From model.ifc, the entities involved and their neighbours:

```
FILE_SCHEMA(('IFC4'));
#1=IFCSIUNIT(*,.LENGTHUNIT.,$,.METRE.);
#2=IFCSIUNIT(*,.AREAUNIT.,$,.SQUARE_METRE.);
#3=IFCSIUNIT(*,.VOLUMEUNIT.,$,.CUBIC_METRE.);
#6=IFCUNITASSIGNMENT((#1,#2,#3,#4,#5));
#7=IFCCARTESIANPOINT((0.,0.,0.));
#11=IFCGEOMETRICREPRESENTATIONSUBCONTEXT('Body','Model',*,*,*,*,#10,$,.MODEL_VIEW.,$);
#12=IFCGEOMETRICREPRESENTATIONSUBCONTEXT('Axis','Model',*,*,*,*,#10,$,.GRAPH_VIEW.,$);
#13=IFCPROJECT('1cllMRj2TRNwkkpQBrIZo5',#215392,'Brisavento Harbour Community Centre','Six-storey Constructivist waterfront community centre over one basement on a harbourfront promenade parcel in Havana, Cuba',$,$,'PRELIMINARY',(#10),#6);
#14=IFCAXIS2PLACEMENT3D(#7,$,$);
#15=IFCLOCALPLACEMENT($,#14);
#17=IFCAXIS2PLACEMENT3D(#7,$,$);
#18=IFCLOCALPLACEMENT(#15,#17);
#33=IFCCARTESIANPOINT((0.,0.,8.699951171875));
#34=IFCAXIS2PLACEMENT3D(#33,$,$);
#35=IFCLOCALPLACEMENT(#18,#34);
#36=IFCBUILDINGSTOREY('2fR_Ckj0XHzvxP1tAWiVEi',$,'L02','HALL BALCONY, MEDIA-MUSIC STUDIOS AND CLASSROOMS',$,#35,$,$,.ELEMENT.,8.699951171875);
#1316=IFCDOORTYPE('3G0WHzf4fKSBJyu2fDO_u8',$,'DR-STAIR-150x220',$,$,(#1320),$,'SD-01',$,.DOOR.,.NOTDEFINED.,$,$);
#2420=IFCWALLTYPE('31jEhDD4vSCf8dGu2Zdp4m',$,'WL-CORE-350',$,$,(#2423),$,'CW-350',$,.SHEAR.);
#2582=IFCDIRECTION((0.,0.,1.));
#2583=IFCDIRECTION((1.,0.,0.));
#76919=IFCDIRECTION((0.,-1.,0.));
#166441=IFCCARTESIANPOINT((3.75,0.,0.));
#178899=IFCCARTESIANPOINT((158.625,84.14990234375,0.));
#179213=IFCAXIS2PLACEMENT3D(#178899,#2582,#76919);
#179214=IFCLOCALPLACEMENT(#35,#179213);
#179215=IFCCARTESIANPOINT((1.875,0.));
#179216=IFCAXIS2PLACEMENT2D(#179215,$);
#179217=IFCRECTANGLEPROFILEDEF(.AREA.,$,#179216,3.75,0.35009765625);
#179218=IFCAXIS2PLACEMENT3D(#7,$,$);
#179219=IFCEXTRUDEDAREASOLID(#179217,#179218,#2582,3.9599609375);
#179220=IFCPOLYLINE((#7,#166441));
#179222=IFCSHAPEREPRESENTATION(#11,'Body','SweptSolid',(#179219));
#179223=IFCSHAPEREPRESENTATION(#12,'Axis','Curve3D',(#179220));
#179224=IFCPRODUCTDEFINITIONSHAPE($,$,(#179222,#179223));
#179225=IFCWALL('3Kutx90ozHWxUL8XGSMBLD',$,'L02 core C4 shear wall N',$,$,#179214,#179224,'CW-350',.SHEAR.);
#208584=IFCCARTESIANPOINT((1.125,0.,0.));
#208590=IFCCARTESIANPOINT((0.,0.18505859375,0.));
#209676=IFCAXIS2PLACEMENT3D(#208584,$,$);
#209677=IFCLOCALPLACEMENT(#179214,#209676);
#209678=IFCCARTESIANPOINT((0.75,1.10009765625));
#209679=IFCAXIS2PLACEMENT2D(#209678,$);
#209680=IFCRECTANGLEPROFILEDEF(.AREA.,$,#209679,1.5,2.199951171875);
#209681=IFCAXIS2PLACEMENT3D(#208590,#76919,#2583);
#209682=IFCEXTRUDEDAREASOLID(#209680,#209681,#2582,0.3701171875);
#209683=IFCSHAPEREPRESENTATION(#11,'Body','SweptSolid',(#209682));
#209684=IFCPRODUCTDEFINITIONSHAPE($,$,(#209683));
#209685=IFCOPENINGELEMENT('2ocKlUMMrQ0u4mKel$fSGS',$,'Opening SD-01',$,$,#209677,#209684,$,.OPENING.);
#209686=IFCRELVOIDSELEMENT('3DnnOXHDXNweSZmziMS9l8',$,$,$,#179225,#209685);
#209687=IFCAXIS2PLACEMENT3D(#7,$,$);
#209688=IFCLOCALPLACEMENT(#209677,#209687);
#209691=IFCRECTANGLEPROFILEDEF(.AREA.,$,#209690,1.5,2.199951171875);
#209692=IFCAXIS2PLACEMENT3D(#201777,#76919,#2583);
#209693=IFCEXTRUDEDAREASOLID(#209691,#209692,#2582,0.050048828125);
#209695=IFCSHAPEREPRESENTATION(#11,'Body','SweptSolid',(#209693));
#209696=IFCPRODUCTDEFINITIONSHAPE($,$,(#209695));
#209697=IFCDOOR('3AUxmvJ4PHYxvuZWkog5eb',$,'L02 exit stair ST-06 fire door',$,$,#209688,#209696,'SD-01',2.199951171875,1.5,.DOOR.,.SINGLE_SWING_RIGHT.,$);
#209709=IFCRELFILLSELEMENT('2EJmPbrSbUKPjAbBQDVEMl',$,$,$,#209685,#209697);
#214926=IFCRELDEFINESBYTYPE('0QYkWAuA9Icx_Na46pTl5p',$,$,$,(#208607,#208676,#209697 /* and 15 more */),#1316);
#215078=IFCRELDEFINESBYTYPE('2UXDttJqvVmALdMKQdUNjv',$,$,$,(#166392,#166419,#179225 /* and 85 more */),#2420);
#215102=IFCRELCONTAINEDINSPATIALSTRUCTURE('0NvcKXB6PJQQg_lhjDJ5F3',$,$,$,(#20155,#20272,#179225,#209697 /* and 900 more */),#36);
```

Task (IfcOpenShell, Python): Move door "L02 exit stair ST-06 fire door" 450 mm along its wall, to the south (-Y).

```python
import ifcopenshell
import ifcopenshell.api.geometry
import ifcopenshell.util.placement
import ifcopenshell.util.unit

model = ifcopenshell.open("model.ifc")
unit_scale = ifcopenshell.util.unit.calculate_unit_scale(model)

door = model.by_guid("3AUxmvJ4PHYxvuZWkog5eb")
opening = door.FillsVoids[0].RelatingOpeningElement
wall = opening.VoidsElements[0].RelatingBuildingElement

wall_matrix = ifcopenshell.util.placement.get_local_placement(wall.ObjectPlacement)
shift = wall_matrix[:3, 0] * 0.45 / unit_scale
before = ifcopenshell.util.placement.get_local_placement(door.ObjectPlacement)[:3, 3].copy()

# The door is placed relative to its opening, so it follows when the opening moves.
matrix = ifcopenshell.util.placement.get_local_placement(opening.ObjectPlacement)
matrix[:3, 3] += shift
ifcopenshell.api.geometry.edit_object_placement(
    model, product=opening, matrix=matrix, is_si=False, should_transform_children=True
)

after = ifcopenshell.util.placement.get_local_placement(door.ObjectPlacement)[:3, 3]
print("door moved by", (after - before).round(3) + 0.0)

model.write("model_v2.ifc")
```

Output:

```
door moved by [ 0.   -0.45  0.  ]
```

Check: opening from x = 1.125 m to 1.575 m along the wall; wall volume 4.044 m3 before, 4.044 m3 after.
